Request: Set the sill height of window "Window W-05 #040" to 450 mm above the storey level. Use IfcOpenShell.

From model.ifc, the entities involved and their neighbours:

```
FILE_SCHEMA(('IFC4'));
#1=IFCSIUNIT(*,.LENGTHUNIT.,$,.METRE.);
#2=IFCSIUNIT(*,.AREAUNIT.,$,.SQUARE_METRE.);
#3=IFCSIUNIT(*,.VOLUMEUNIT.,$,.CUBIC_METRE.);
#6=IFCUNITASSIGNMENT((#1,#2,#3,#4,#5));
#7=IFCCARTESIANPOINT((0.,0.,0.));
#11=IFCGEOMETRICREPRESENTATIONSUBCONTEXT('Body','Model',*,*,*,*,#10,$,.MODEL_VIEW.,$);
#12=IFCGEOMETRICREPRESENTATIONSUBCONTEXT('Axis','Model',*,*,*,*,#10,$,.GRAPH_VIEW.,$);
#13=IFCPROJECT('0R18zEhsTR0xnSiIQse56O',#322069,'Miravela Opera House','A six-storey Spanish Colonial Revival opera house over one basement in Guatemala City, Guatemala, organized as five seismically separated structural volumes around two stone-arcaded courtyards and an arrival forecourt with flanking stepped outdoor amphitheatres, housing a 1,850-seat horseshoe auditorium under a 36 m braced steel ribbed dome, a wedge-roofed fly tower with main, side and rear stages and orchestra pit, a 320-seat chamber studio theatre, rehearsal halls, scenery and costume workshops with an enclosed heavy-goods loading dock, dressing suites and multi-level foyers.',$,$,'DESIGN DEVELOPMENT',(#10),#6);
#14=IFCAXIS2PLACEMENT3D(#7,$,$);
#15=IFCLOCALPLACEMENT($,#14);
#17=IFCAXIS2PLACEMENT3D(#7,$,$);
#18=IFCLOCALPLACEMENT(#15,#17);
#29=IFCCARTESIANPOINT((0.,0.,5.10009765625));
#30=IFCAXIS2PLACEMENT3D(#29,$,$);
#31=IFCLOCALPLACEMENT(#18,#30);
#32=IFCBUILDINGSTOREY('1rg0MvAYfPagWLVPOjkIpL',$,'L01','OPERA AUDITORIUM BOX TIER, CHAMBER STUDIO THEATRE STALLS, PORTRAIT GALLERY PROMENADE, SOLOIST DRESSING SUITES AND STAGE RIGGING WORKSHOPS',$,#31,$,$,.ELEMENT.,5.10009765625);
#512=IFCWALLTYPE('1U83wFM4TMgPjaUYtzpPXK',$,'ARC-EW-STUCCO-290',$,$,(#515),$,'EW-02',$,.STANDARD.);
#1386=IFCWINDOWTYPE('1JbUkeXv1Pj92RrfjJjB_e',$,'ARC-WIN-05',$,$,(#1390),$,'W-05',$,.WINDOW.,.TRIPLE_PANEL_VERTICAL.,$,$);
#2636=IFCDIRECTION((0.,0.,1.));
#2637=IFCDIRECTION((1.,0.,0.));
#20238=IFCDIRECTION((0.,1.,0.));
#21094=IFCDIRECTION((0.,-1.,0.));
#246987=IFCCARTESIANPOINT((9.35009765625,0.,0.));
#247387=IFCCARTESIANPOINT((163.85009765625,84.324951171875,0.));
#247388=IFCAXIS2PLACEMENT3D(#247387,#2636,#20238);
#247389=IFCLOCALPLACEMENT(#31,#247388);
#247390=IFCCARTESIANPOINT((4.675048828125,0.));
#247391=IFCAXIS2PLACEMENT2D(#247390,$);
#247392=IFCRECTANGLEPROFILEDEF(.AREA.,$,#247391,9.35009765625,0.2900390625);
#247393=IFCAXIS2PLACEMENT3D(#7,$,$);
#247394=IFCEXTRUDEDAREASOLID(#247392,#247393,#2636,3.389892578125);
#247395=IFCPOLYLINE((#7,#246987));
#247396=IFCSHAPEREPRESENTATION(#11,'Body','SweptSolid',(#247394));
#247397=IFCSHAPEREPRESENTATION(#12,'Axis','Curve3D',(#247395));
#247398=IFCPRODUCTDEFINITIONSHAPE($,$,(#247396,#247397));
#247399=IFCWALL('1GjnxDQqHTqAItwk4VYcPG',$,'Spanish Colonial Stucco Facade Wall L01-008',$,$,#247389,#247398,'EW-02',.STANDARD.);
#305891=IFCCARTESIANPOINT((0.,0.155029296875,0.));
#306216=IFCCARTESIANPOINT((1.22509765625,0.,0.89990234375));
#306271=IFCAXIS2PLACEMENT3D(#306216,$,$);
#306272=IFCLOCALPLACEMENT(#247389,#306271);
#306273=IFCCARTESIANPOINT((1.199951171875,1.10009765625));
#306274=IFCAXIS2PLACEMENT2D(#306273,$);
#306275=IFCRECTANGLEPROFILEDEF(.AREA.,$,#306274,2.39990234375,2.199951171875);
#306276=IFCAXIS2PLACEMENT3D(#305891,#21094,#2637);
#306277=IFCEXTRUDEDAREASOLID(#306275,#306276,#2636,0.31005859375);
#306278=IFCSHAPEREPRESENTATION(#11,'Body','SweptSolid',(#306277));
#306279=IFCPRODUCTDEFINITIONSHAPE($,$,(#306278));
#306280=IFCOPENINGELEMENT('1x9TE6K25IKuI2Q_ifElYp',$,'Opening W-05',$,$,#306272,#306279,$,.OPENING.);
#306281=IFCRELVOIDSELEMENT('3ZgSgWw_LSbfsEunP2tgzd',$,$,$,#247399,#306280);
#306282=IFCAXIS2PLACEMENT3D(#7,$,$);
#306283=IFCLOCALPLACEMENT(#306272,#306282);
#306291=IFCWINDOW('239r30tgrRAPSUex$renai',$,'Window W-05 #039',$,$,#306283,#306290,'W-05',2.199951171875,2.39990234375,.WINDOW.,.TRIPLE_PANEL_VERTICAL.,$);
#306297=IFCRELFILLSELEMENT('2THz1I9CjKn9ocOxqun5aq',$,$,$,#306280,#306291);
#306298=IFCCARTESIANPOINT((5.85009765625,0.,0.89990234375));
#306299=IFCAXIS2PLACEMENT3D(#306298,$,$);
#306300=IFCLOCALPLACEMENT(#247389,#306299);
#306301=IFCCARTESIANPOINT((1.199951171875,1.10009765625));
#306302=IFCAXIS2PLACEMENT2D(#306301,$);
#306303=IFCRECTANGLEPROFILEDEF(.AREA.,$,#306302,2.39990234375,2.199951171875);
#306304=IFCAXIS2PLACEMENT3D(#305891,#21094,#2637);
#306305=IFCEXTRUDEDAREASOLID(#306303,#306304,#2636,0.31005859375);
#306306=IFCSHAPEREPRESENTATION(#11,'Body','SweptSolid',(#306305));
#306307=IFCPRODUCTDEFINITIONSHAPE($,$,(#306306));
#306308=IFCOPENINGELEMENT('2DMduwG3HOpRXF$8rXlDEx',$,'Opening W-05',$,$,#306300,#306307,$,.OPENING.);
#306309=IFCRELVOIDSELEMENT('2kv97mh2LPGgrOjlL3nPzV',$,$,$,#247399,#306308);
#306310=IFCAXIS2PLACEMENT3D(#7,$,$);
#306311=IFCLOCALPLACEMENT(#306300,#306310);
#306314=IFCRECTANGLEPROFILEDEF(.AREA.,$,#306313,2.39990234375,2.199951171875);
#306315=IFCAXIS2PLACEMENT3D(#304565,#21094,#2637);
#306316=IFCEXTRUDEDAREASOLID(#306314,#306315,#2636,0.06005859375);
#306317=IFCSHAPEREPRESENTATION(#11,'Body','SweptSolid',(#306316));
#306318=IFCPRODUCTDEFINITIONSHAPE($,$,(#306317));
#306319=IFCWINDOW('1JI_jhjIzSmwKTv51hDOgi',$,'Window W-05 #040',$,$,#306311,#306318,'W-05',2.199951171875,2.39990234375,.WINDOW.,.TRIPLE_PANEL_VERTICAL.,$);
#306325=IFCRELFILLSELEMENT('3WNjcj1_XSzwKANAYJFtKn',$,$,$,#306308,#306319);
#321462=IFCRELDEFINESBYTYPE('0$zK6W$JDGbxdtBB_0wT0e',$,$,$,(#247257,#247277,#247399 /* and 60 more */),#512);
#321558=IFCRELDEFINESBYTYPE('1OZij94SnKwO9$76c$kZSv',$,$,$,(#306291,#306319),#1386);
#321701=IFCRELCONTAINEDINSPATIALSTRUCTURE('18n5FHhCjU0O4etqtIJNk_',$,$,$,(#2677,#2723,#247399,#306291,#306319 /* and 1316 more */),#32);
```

```python
import numpy as np
import ifcopenshell
import ifcopenshell.api.geometry
import ifcopenshell.geom
import ifcopenshell.util.element
import ifcopenshell.util.placement
import ifcopenshell.util.shape
import ifcopenshell.util.unit

model = ifcopenshell.open("model.ifc")
unit_scale = ifcopenshell.util.unit.calculate_unit_scale(model)

window = model.by_id(306319)
opening = window.FillsVoids[0].RelatingOpeningElement
storey = ifcopenshell.util.element.get_container(window, ifc_class="IfcBuildingStorey")
level = ifcopenshell.util.placement.get_local_placement(storey.ObjectPlacement)[2, 3]

# The opening's origin need not be at the sill, so measure its lowest point.
shape = ifcopenshell.geom.create_shape(ifcopenshell.geom.settings(), opening)
bottom = ifcopenshell.util.shape.get_shape_bottom_elevation(shape, shape.geometry) / unit_scale
dz = level + 0.45 - bottom

shift = np.array([0.0, 0.0, dz])
# The window is placed relative to its opening, so it follows when the opening moves.
matrix = ifcopenshell.util.placement.get_local_placement(opening.ObjectPlacement)
matrix[:3, 3] += shift
ifcopenshell.api.geometry.edit_object_placement(
    model, product=opening, matrix=matrix, is_si=False, should_transform_children=True
)

print(f"moved by {dz * unit_scale:+.3f} m")

model.write("model_edited.ifc")
```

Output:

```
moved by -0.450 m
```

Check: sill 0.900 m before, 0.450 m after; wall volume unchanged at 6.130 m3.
